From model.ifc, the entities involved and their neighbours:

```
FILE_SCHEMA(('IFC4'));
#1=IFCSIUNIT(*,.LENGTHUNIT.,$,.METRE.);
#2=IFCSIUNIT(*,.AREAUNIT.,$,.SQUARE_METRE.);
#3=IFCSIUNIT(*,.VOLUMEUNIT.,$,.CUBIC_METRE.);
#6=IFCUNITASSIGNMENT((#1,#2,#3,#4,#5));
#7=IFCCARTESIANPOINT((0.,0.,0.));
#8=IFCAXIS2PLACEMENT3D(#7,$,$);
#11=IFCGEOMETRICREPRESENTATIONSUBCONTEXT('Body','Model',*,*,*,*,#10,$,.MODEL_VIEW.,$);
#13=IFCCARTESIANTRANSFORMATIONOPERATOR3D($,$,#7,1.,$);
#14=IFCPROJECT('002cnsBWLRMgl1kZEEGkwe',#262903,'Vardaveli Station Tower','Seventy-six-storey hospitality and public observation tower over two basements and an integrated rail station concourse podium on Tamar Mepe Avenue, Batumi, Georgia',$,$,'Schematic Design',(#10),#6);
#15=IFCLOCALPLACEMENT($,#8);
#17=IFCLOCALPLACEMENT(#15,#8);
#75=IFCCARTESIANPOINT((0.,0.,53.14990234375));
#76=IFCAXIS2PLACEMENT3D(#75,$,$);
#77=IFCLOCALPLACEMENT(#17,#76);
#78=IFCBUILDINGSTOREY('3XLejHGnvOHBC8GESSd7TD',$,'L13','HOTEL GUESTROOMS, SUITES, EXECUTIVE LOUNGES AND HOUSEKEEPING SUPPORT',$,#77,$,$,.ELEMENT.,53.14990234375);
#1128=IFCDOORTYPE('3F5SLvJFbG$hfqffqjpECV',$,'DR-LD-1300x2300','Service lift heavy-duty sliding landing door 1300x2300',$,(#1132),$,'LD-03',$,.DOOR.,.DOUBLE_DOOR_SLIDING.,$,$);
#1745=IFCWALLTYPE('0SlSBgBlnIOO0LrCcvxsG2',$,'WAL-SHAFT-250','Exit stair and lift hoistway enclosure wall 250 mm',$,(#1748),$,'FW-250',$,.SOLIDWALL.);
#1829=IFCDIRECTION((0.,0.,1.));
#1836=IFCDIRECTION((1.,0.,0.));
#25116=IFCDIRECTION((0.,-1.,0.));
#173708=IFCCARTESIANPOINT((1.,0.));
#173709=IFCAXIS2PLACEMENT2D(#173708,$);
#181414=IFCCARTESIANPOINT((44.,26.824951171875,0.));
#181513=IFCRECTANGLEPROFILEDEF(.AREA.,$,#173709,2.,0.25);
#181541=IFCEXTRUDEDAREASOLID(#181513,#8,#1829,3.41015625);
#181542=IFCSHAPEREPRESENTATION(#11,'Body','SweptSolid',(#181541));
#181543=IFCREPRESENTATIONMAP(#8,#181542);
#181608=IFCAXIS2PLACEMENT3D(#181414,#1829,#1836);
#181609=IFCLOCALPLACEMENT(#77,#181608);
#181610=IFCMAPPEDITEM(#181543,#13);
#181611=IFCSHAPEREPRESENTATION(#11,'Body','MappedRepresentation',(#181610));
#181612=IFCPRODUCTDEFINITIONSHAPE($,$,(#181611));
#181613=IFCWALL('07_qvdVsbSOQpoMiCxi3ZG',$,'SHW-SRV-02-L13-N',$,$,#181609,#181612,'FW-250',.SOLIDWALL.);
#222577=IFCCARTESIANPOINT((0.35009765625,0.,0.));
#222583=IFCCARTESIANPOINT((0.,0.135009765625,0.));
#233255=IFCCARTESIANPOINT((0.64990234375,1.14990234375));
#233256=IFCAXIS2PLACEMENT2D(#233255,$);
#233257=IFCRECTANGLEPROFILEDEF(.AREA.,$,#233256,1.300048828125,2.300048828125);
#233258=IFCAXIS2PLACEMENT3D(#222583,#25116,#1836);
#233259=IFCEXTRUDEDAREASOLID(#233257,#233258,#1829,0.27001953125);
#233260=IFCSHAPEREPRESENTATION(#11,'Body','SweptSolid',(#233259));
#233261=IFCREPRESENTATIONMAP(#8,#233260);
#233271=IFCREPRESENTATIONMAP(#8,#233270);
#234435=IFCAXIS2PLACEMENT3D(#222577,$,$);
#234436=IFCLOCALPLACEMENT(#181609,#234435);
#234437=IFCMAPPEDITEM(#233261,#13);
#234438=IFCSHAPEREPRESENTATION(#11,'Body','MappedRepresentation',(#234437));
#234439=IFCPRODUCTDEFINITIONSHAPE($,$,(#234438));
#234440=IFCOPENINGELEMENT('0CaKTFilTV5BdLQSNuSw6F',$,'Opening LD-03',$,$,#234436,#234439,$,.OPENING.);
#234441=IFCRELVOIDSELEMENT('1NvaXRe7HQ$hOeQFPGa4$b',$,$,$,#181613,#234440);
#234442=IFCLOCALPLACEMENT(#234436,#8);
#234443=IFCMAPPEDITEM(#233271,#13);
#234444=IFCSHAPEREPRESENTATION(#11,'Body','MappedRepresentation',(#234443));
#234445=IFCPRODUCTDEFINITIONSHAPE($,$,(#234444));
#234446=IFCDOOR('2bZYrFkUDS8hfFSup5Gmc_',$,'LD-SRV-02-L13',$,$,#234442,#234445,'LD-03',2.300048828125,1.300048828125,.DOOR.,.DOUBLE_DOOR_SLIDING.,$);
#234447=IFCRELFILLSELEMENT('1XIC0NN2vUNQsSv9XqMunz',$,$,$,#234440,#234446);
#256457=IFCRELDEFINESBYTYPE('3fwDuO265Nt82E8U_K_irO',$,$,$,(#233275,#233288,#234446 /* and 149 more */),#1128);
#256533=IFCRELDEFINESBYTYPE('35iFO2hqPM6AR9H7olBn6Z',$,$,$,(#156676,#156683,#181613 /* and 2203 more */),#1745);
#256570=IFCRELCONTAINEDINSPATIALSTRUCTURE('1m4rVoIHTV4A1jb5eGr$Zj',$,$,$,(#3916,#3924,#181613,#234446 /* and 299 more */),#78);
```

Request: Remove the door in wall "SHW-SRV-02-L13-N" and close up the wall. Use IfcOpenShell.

```python
import ifcopenshell
import ifcopenshell.api.feature
import ifcopenshell.api.root
import ifcopenshell.geom
import ifcopenshell.util.shape

model = ifcopenshell.open("model.ifc")
settings = ifcopenshell.geom.settings()


def volume(element):
    """Net volume in cubic metres, openings subtracted."""
    shape = ifcopenshell.geom.create_shape(settings, element)
    return ifcopenshell.util.shape.get_volume(shape.geometry)


door = model.by_guid("2bZYrFkUDS8hfFSup5Gmc_")
opening = door.FillsVoids[0].RelatingOpeningElement
wall = opening.VoidsElements[0].RelatingBuildingElement
before = volume(wall)

ifcopenshell.api.root.remove_product(model, product=door)
ifcopenshell.api.feature.remove_feature(model, feature=opening)

after = volume(wall)

print(f"wall volume {before:.3f} -> {after:.3f} m3")

model.write("model_v2.ifc")
```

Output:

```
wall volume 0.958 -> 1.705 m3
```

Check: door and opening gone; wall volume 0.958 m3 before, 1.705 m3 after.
